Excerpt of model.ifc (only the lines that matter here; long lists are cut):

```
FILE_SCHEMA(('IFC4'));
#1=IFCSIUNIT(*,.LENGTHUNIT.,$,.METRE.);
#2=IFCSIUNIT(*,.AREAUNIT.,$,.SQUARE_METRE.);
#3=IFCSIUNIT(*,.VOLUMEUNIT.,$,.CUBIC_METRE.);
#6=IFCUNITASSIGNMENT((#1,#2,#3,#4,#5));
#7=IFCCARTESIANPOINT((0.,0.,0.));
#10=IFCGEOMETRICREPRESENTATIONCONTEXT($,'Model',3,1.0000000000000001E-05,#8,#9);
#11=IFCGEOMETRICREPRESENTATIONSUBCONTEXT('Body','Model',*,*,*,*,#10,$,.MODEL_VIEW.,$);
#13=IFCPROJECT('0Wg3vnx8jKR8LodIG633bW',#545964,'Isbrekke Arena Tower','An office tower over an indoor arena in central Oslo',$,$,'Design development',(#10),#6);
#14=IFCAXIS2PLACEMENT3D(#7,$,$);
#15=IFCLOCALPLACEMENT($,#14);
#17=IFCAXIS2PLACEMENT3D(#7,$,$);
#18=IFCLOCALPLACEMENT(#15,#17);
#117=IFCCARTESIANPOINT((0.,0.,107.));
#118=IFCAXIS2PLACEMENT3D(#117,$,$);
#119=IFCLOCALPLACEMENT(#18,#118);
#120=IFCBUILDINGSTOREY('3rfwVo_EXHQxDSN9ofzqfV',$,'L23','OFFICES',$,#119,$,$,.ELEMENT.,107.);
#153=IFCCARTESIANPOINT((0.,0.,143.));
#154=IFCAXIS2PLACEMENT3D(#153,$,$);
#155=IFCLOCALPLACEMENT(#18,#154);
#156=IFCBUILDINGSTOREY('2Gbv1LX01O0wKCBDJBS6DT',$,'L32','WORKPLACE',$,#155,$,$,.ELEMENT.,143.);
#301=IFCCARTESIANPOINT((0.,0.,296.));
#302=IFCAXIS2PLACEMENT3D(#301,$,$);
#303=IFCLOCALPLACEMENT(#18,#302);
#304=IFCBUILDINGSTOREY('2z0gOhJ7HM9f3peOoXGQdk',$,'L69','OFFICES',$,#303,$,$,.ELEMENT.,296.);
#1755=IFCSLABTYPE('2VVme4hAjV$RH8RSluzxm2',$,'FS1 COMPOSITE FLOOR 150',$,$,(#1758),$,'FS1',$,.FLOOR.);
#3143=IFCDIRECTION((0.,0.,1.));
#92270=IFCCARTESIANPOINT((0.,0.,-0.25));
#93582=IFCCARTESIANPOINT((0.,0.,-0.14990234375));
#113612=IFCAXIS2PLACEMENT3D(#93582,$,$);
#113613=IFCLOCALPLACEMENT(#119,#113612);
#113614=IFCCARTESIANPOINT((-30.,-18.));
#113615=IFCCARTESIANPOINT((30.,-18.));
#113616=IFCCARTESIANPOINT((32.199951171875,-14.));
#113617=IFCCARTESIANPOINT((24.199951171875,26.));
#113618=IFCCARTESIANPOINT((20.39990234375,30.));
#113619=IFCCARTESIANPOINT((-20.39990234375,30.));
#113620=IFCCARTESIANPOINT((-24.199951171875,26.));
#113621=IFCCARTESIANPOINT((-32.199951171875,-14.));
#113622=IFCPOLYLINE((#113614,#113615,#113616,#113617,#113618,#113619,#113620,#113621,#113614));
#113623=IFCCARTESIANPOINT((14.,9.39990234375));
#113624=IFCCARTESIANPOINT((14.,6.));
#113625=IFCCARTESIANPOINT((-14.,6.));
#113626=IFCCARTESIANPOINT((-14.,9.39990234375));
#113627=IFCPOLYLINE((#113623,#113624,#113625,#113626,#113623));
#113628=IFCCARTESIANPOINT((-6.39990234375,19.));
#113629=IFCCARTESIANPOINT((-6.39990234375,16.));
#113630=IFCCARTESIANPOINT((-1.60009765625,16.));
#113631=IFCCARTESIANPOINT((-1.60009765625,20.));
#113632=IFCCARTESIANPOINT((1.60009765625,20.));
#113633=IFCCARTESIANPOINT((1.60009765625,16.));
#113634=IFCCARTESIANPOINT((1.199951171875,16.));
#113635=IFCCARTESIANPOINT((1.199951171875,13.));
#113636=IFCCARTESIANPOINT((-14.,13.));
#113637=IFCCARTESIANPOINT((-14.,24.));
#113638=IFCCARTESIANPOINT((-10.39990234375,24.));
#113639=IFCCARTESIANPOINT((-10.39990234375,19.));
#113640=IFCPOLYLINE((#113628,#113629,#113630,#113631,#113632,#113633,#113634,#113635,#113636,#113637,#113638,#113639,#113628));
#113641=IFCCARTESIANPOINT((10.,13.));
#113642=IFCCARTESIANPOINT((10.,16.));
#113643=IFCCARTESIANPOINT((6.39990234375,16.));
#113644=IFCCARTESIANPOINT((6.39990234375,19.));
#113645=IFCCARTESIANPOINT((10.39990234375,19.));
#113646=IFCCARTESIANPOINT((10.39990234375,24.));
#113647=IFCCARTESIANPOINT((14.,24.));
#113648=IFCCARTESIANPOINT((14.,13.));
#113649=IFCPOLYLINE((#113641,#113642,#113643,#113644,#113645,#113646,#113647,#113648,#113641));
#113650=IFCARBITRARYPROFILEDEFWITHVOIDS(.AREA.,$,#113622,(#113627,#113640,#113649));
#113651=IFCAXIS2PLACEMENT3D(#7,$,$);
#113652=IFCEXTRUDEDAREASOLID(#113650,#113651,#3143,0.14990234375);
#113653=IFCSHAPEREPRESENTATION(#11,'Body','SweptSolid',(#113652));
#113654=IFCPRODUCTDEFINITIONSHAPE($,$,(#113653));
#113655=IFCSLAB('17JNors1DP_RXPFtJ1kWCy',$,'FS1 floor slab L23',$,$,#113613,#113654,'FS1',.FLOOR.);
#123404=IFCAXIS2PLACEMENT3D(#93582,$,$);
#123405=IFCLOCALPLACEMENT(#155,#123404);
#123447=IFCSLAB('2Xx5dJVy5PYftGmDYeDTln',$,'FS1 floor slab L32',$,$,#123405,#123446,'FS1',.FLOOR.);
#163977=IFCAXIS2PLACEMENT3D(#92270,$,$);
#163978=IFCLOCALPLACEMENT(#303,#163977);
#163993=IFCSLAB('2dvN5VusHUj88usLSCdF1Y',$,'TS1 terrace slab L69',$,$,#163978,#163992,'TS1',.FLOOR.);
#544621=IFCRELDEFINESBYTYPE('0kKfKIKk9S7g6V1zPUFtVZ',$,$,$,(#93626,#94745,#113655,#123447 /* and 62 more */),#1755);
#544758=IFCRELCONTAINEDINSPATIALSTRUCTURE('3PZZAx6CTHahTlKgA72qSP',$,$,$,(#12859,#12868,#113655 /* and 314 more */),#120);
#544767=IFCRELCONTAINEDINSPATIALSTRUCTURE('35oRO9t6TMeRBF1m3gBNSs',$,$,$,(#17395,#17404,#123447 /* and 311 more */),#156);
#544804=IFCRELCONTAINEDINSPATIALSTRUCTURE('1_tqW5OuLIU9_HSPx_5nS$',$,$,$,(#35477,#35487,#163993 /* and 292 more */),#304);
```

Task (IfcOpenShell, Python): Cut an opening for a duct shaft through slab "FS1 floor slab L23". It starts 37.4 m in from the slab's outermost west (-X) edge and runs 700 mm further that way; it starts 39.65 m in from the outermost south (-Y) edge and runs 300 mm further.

```python
import numpy as np
import ifcopenshell
import ifcopenshell.api.feature
import ifcopenshell.api.geometry
import ifcopenshell.api.root
import ifcopenshell.geom
import ifcopenshell.util.placement
import ifcopenshell.util.representation
import ifcopenshell.util.shape
import ifcopenshell.util.unit

model = ifcopenshell.open("model.ifc")
unit_scale = ifcopenshell.util.unit.calculate_unit_scale(model)
settings = ifcopenshell.geom.settings()


def volume(element):
    """Net volume in cubic metres, openings subtracted."""
    shape = ifcopenshell.geom.create_shape(settings, element)
    return ifcopenshell.util.shape.get_volume(shape.geometry)


slab = model.by_id(113655)
before = volume(slab)

# Extent in the slab's own axes, in metres. The edges named are its -X and -Y sides.
slab_shape = ifcopenshell.geom.create_shape(settings, slab)
vertices = ifcopenshell.util.shape.get_vertices(slab_shape.geometry)
x_min, y_min, bottom = vertices.min(axis=0)
top = vertices[:, 2].max()

opening = ifcopenshell.api.root.create_entity(model, ifc_class="IfcOpeningElement", name="Duct shaft opening", predefined_type="OPENING")
context = ifcopenshell.util.representation.get_context(model, "Model", "Body", "MODEL_VIEW")
width, depth = 0.7, 0.3
outline = [(0.0, 0.0), (width, 0.0), (width, depth), (0.0, depth), (0.0, 0.0)]
# Overshoot both faces by 50 mm so the cut is clean.
shape = ifcopenshell.api.geometry.add_slab_representation(
    model, context=context, depth=top - bottom + 0.1, polyline=outline
)
ifcopenshell.api.geometry.assign_representation(model, product=opening, representation=shape)

matrix = ifcopenshell.util.placement.get_local_placement(slab.ObjectPlacement)
matrix[:, 3] = matrix @ np.append(np.array([x_min + 37.4, y_min + 39.65, bottom - 0.05]) / unit_scale, 1.0)
ifcopenshell.api.geometry.edit_object_placement(model, product=opening, matrix=matrix, is_si=False)
ifcopenshell.api.feature.add_feature(model, feature=opening, element=slab)

after = volume(slab)

print(f"slab volume {before:.3f} -> {after:.3f} m3")

model.write("model_updated.ifc")
```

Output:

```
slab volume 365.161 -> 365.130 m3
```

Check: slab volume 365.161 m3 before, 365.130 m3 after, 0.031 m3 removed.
